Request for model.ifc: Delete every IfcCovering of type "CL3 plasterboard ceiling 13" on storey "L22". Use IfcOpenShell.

First a look at what the model holds.

```python
import ifcopenshell
import ifcopenshell.util.element

model = ifcopenshell.open("model.ifc")
print(model.schema)
storey = next(s for s in model.by_type("IfcBuildingStorey") if s.Name == "L22")
coverings = [e for e in ifcopenshell.util.element.get_decomposition(storey) if e.is_a("IfcCovering")]
seen = {}
for e in coverings:
    element_type = ifcopenshell.util.element.get_type(e)
    name = element_type.Name if element_type not in (None, e) else None
    seen[name] = seen.get(name, 0) + 1
for name, count in sorted(seen.items(), key=str):
    print(count, "x", name)
```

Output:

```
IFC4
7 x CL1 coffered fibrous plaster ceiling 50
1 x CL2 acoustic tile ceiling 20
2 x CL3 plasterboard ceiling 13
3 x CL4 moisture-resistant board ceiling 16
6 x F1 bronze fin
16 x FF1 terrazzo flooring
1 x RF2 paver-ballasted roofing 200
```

```python
import ifcopenshell
import ifcopenshell.api.root
import ifcopenshell.util.element

model = ifcopenshell.open("model.ifc")

storey = next(s for s in model.by_type("IfcBuildingStorey") if s.Name == "L22")
coverings = [e for e in ifcopenshell.util.element.get_decomposition(storey) if e.is_a("IfcCovering")]
targets = [e for e in coverings if (t := ifcopenshell.util.element.get_type(e)) not in (None, e) and t.Name == "CL3 plasterboard ceiling 13"]

for e in targets:
    ifcopenshell.api.root.remove_product(model, product=e)
print(len(targets), "removed")

model.write("model_edited.ifc")
```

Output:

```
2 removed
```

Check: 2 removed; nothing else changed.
